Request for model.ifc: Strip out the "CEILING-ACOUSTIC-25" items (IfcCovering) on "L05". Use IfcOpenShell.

First a look at what the model holds.

```python
import ifcopenshell
import ifcopenshell.util.element

model = ifcopenshell.open("model.ifc")
print(model.schema)
storey = next(s for s in model.by_type("IfcBuildingStorey") if s.Name == "L05")
coverings = [e for e in ifcopenshell.util.element.get_decomposition(storey) if e.is_a("IfcCovering")]
seen = {}
for e in coverings:
    element_type = ifcopenshell.util.element.get_type(e)
    name = element_type.Name if element_type not in (None, e) else None
    seen[name] = seen.get(name, 0) + 1
for name, count in sorted(seen.items(), key=str):
    print(count, "x", name)
```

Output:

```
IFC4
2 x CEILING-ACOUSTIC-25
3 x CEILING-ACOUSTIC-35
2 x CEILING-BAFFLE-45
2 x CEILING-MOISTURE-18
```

```python
import ifcopenshell
import ifcopenshell.api.root
import ifcopenshell.util.element

model = ifcopenshell.open("model.ifc")

storey = next(s for s in model.by_type("IfcBuildingStorey") if s.Name == "L05")
coverings = [e for e in ifcopenshell.util.element.get_decomposition(storey) if e.is_a("IfcCovering")]
targets = [e for e in coverings if (t := ifcopenshell.util.element.get_type(e)) not in (None, e) and t.Name == "CEILING-ACOUSTIC-25"]

for e in targets:
    ifcopenshell.api.root.remove_product(model, product=e)
print(len(targets), "removed")

model.write("model_v2.ifc")
```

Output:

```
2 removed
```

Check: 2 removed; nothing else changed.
